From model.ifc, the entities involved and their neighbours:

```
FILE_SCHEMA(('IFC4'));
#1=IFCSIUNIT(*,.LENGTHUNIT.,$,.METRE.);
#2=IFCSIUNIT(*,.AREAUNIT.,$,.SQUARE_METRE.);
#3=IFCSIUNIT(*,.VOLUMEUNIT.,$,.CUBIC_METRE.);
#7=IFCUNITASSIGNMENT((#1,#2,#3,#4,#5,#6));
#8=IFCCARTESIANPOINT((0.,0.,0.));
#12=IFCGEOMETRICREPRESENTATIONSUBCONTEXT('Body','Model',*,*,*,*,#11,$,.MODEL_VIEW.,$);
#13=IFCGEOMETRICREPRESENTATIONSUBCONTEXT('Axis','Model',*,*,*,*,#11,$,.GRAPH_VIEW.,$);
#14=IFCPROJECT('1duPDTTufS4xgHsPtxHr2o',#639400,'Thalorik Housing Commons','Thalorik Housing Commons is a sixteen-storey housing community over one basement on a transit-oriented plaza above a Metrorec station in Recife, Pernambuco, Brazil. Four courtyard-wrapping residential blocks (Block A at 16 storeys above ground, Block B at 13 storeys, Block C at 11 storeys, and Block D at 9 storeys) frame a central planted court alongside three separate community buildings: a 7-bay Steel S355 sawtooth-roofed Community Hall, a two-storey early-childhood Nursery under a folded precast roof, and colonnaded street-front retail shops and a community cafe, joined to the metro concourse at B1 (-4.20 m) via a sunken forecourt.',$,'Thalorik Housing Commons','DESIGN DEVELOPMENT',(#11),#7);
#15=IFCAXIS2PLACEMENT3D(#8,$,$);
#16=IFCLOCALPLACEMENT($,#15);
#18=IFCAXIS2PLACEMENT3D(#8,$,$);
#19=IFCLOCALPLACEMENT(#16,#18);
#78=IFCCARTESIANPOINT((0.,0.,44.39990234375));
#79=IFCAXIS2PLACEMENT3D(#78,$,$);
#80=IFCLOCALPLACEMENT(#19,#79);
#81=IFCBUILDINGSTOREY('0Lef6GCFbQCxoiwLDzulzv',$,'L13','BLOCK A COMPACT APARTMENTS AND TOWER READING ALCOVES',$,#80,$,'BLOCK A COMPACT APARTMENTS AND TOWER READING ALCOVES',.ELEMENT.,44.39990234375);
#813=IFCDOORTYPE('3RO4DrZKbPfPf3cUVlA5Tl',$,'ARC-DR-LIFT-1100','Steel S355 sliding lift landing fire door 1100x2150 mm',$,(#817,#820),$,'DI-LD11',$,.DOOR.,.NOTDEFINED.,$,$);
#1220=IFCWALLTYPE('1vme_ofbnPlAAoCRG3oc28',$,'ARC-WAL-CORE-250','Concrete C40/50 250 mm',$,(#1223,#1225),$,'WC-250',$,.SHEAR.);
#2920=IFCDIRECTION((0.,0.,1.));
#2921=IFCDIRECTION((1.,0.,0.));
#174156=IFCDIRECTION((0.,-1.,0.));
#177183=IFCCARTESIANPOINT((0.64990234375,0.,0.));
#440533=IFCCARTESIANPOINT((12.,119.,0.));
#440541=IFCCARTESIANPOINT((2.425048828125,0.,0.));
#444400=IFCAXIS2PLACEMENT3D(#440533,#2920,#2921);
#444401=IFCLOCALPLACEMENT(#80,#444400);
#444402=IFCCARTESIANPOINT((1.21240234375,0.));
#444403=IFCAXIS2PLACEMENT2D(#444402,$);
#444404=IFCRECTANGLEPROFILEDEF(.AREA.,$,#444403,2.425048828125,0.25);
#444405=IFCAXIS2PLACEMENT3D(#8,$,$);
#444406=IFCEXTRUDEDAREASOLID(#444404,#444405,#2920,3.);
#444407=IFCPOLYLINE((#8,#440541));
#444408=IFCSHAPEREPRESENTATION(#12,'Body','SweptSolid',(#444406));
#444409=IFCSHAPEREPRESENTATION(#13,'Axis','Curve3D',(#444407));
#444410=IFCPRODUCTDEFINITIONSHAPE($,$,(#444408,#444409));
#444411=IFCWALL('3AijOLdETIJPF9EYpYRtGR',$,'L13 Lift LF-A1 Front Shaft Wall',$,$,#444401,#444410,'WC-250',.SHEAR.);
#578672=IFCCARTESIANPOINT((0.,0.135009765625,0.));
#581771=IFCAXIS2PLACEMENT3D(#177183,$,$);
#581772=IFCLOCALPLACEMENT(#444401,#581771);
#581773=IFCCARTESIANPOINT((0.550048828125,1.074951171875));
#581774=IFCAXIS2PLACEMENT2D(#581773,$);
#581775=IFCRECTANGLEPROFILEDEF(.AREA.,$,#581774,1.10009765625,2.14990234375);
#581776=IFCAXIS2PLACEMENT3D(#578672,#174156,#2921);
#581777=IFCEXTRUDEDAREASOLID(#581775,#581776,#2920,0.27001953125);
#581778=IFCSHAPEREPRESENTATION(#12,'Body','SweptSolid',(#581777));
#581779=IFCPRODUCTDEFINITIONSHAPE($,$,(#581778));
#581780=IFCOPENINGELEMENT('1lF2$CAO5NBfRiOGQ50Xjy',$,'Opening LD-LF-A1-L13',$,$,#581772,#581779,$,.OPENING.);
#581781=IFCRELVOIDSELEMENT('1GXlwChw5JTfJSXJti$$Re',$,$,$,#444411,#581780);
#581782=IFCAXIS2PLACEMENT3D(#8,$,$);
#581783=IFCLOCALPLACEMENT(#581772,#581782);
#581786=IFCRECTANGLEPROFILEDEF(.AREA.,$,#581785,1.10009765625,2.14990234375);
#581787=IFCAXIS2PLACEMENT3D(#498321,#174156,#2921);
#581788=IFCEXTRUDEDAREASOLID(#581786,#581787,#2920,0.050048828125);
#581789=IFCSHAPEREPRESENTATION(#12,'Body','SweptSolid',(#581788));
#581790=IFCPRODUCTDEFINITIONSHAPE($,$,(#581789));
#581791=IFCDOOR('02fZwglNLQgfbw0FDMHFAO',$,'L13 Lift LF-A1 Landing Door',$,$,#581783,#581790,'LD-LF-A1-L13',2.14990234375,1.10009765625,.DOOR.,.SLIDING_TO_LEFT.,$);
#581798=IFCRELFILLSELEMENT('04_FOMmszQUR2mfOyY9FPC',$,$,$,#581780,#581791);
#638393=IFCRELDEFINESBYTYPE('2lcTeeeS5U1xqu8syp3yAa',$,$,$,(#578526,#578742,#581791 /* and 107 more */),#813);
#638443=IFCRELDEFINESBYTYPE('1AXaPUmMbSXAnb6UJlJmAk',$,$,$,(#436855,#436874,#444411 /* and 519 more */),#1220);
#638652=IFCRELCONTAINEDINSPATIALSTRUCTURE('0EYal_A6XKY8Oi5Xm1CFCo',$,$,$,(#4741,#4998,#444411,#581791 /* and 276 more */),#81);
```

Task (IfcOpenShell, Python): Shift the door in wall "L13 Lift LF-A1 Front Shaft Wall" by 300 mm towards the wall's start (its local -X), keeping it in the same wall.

```python
import ifcopenshell
import ifcopenshell.api.geometry
import ifcopenshell.util.placement
import ifcopenshell.util.unit

model = ifcopenshell.open("model.ifc")
unit_scale = ifcopenshell.util.unit.calculate_unit_scale(model)

door = model.by_guid("02fZwglNLQgfbw0FDMHFAO")
opening = door.FillsVoids[0].RelatingOpeningElement
wall = opening.VoidsElements[0].RelatingBuildingElement

wall_matrix = ifcopenshell.util.placement.get_local_placement(wall.ObjectPlacement)
shift = wall_matrix[:3, 0] * -0.3 / unit_scale
before = ifcopenshell.util.placement.get_local_placement(door.ObjectPlacement)[:3, 3].copy()

# The door is placed relative to its opening, so it follows when the opening moves.
matrix = ifcopenshell.util.placement.get_local_placement(opening.ObjectPlacement)
matrix[:3, 3] += shift
ifcopenshell.api.geometry.edit_object_placement(
    model, product=opening, matrix=matrix, is_si=False, should_transform_children=True
)

after = ifcopenshell.util.placement.get_local_placement(door.ObjectPlacement)[:3, 3]
print("door moved by", (after - before).round(3) + 0.0)

model.write("model-out.ifc")
```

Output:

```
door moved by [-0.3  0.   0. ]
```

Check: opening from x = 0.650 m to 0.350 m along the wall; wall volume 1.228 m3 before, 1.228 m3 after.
